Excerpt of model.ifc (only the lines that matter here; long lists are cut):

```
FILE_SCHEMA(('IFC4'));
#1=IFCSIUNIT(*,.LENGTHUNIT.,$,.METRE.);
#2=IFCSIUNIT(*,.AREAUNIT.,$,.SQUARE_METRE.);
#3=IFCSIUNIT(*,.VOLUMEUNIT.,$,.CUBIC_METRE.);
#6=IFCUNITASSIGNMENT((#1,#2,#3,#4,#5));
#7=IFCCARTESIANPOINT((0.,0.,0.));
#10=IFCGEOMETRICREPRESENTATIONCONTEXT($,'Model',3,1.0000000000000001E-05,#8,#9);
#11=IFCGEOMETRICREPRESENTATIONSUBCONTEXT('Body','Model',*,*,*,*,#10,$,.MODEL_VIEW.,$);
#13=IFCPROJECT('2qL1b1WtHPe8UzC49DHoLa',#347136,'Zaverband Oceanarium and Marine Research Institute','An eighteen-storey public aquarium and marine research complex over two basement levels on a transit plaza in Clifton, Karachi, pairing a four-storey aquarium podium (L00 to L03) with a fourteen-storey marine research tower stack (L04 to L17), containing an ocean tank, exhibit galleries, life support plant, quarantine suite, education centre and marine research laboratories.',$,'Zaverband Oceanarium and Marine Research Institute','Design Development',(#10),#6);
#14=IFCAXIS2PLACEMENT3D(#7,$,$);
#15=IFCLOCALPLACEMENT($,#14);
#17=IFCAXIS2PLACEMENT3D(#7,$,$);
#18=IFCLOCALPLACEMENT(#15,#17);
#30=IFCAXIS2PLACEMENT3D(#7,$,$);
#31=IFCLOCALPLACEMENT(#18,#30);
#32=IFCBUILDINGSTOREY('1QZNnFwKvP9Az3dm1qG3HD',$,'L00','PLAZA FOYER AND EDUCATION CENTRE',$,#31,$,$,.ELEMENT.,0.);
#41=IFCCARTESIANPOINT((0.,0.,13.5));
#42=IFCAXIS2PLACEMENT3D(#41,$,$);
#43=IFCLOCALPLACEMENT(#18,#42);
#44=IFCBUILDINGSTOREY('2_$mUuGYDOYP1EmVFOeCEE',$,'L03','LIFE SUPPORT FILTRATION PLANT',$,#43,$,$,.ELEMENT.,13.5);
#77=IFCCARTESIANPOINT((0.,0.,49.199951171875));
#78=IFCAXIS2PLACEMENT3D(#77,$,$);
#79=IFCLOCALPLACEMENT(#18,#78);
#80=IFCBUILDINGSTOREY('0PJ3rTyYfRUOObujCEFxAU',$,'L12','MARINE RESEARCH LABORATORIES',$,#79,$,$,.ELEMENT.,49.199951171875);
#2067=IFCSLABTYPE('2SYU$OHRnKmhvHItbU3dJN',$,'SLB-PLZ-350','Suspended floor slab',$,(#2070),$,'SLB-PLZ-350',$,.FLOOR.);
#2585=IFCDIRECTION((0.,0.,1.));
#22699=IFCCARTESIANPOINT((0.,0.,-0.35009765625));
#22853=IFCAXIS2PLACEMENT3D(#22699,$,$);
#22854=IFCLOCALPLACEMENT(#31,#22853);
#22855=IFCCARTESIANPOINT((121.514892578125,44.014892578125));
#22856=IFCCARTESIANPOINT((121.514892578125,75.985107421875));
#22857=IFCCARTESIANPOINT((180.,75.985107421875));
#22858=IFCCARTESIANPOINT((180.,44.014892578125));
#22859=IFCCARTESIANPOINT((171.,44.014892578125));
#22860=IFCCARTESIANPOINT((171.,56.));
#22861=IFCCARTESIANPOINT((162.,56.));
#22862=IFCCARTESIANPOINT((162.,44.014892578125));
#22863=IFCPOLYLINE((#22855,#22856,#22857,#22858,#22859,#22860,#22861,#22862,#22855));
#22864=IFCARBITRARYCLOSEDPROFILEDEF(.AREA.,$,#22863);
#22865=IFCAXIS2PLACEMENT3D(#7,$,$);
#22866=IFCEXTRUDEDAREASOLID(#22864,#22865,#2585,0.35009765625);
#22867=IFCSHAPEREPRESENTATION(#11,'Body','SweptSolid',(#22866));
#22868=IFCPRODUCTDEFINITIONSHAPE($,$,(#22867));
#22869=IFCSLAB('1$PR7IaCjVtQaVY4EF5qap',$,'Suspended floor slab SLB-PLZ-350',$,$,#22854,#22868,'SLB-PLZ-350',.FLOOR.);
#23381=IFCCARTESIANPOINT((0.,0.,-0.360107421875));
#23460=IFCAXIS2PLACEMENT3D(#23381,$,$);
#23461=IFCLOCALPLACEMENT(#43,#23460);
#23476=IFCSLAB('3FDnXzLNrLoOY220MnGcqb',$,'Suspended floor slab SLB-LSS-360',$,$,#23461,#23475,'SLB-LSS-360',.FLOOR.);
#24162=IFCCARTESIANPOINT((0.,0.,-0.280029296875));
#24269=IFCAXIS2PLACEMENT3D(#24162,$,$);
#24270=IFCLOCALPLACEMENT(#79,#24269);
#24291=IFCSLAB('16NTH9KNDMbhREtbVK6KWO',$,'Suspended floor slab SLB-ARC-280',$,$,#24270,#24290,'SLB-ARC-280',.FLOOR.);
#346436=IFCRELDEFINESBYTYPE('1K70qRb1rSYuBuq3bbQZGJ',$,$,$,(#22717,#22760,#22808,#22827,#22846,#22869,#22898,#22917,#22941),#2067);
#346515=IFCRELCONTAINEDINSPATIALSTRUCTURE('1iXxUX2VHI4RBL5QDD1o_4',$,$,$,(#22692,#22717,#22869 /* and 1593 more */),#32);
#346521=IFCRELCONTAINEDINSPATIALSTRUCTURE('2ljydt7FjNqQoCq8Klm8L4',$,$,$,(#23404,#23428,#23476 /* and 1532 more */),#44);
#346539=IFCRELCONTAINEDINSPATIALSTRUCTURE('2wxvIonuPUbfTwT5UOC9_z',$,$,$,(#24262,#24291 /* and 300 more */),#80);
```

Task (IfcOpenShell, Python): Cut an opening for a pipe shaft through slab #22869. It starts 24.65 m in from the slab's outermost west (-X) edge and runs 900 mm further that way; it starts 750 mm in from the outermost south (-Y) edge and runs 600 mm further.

```python
import numpy as np
import ifcopenshell
import ifcopenshell.api.feature
import ifcopenshell.api.geometry
import ifcopenshell.api.root
import ifcopenshell.geom
import ifcopenshell.util.placement
import ifcopenshell.util.representation
import ifcopenshell.util.shape
import ifcopenshell.util.unit

model = ifcopenshell.open("model.ifc")
unit_scale = ifcopenshell.util.unit.calculate_unit_scale(model)
settings = ifcopenshell.geom.settings()


def volume(element):
    """Net volume in cubic metres, openings subtracted."""
    shape = ifcopenshell.geom.create_shape(settings, element)
    return ifcopenshell.util.shape.get_volume(shape.geometry)


slab = model.by_guid("1$PR7IaCjVtQaVY4EF5qap")
before = volume(slab)

# Extent in the slab's own axes, in metres. The edges named are its -X and -Y sides.
slab_shape = ifcopenshell.geom.create_shape(settings, slab)
vertices = ifcopenshell.util.shape.get_vertices(slab_shape.geometry)
x_min, y_min, bottom = vertices.min(axis=0)
top = vertices[:, 2].max()

opening = ifcopenshell.api.root.create_entity(model, ifc_class="IfcOpeningElement", name="Pipe shaft opening", predefined_type="OPENING")
context = ifcopenshell.util.representation.get_context(model, "Model", "Body", "MODEL_VIEW")
width, depth = 0.9, 0.6
outline = [(0.0, 0.0), (width, 0.0), (width, depth), (0.0, depth), (0.0, 0.0)]
# Overshoot both faces by 50 mm so the cut is clean.
shape = ifcopenshell.api.geometry.add_slab_representation(
    model, context=context, depth=top - bottom + 0.1, polyline=outline
)
ifcopenshell.api.geometry.assign_representation(model, product=opening, representation=shape)

matrix = ifcopenshell.util.placement.get_local_placement(slab.ObjectPlacement)
matrix[:, 3] = matrix @ np.append(np.array([x_min + 24.65, y_min + 0.75, bottom - 0.05]) / unit_scale, 1.0)
ifcopenshell.api.geometry.edit_object_placement(model, product=opening, matrix=matrix, is_si=False)
ifcopenshell.api.feature.add_feature(model, feature=opening, element=slab)

after = volume(slab)

print(f"slab volume {before:.3f} -> {after:.3f} m3")

model.write("model_edited.ifc")
```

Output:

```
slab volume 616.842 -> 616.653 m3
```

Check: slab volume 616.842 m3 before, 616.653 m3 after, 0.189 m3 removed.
